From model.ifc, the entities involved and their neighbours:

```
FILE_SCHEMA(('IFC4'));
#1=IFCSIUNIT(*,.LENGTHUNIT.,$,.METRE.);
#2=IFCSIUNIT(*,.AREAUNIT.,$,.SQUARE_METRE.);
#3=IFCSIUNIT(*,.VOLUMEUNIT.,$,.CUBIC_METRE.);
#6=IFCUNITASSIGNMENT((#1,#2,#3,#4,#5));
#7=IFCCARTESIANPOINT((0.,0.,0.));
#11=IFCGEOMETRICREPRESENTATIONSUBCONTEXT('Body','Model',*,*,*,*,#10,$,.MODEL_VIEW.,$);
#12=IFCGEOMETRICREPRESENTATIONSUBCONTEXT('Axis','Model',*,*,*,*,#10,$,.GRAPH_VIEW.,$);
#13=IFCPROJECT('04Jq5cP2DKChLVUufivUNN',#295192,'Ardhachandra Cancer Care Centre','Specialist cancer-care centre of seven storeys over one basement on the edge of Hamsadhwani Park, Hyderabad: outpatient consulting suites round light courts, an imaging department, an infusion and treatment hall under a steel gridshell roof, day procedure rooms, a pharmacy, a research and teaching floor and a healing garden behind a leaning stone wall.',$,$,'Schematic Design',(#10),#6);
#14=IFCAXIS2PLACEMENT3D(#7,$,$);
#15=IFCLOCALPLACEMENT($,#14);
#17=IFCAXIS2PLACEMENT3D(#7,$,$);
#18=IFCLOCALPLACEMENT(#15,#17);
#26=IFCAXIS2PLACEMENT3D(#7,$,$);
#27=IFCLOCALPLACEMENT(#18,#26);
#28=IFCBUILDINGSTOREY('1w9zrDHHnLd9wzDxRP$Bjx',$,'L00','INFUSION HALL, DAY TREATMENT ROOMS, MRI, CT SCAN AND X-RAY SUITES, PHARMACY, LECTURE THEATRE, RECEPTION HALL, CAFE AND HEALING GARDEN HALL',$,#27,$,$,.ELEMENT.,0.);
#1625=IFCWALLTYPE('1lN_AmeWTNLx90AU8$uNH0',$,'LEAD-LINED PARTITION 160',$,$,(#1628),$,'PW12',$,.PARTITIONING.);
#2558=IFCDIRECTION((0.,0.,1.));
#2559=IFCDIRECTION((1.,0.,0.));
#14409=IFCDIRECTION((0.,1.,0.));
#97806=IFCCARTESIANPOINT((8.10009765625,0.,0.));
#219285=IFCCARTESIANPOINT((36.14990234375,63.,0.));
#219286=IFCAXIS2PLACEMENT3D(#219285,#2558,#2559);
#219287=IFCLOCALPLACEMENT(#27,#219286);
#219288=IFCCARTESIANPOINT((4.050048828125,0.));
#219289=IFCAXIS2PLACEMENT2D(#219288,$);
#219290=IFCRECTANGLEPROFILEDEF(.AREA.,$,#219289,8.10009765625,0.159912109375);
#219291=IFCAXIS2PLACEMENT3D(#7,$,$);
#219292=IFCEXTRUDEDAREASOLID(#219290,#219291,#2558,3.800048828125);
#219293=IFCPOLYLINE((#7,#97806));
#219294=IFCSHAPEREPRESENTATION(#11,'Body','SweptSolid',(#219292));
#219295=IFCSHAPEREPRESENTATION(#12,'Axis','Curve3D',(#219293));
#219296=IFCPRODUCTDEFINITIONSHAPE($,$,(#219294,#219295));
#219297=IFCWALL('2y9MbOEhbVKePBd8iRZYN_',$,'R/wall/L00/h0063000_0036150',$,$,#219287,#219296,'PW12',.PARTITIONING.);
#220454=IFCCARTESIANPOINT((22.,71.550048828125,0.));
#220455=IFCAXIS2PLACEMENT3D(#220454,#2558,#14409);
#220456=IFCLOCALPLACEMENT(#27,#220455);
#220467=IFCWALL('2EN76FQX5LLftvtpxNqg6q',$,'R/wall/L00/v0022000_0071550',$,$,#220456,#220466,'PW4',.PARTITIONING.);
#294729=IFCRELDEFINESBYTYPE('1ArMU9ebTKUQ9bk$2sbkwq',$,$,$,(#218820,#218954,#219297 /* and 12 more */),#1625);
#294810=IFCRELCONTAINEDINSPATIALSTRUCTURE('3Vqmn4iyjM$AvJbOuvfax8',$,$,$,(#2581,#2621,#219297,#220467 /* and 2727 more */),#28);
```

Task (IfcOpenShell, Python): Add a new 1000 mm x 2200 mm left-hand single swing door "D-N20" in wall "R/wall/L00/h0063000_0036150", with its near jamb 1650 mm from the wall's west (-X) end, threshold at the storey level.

```python
import numpy as np
import ifcopenshell
import ifcopenshell.api.feature
import ifcopenshell.api.geometry
import ifcopenshell.api.root
import ifcopenshell.api.spatial
import ifcopenshell.geom
import ifcopenshell.util.element
import ifcopenshell.util.placement
import ifcopenshell.util.representation
import ifcopenshell.util.shape
import ifcopenshell.util.unit

model = ifcopenshell.open("model.ifc")
unit_scale = ifcopenshell.util.unit.calculate_unit_scale(model)
settings = ifcopenshell.geom.settings()


def volume(element):
    """Net volume in cubic metres, openings subtracted."""
    shape = ifcopenshell.geom.create_shape(settings, element)
    return ifcopenshell.util.shape.get_volume(shape.geometry)


wall = model.by_id(219297)
storey = ifcopenshell.util.element.get_container(wall, ifc_class="IfcBuildingStorey")
context = ifcopenshell.util.representation.get_context(model, "Model", "Body", "MODEL_VIEW")
before = volume(wall)

width, height, from_end, sill = 1, 2.2, 1.65, 0.0  # metres

# The wall runs along its own X axis, and the end named is its -X end.
wall_shape = ifcopenshell.geom.create_shape(settings, wall)
x, y, z = ifcopenshell.util.shape.get_vertices(wall_shape.geometry).T
start = x.min() + from_end
face, thickness = float(y.min()), float(y.max() - y.min())
wall_matrix = ifcopenshell.util.placement.get_local_placement(wall.ObjectPlacement)
level = ifcopenshell.util.placement.get_local_placement(storey.ObjectPlacement)[2, 3]


def in_wall(x, y):
    """Placement at x, y metres in the wall's axes, at sill height."""
    matrix = wall_matrix.copy()
    matrix[:, 3] = wall_matrix @ np.array([x / unit_scale, y / unit_scale, 0.0, 1.0])
    matrix[2, 3] = level + sill / unit_scale
    return matrix


# Opening: a box that overshoots both wall faces by 50 mm.
opening = ifcopenshell.api.root.create_entity(model, ifc_class="IfcOpeningElement", predefined_type="OPENING")
box = ifcopenshell.api.geometry.add_wall_representation(
    model, context=context, length=width, height=height, thickness=thickness + 0.1
)
ifcopenshell.api.geometry.assign_representation(model, product=opening, representation=box)
ifcopenshell.api.geometry.edit_object_placement(model, product=opening, matrix=in_wall(start, face - 0.05), is_si=False)
ifcopenshell.api.feature.add_feature(model, feature=opening, element=wall)

door = ifcopenshell.api.root.create_entity(model, ifc_class="IfcDoor", name="D-N20", predefined_type="DOOR")
door.OverallWidth, door.OverallHeight = width / unit_scale, height / unit_scale
door.OperationType = "SINGLE_SWING_LEFT"
body = ifcopenshell.api.geometry.add_door_representation(
    model,
    context=context,
    overall_width=door.OverallWidth,
    overall_height=door.OverallHeight,
    operation_type="SINGLE_SWING_LEFT",
    lining_properties={"LiningDepth": thickness / unit_scale, "ThresholdDepth": thickness / unit_scale},
)
ifcopenshell.api.geometry.assign_representation(model, product=door, representation=body)
ifcopenshell.api.spatial.assign_container(model, products=[door], relating_structure=storey)
ifcopenshell.api.feature.add_filling(model, opening=opening, element=door)

# The lining spans the wall, so the door starts at the wall face.
ifcopenshell.api.geometry.edit_object_placement(model, product=door, matrix=in_wall(start, face), is_si=False)

after = volume(wall)

print(f"wall volume {before:.3f} -> {after:.3f} m3")

model.write("model_v2.ifc")
```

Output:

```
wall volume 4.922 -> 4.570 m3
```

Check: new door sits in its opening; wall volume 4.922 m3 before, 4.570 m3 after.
